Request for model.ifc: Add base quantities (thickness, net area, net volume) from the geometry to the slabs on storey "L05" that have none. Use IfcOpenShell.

First a look at what the model holds.

```python
import ifcopenshell
import ifcopenshell.util.element
import ifcopenshell.util.unit

model = ifcopenshell.open("model.ifc")
print(model.schema)
for unit_type in ("LENGTHUNIT", "AREAUNIT", "VOLUMEUNIT"):
    print(unit_type, ifcopenshell.util.unit.calculate_unit_scale(model, unit_type))
storey = next(s for s in model.by_type("IfcBuildingStorey") if s.Name == "L05")
slabs = [e for e in ifcopenshell.util.element.get_decomposition(storey) if e.is_a("IfcSlab")]
for e in sorted(slabs, key=lambda e: e.id()):
    print(e.id(), e.is_a(), e.Name, list(ifcopenshell.util.element.get_psets(e, qtos_only=True)), sep=" | ")
```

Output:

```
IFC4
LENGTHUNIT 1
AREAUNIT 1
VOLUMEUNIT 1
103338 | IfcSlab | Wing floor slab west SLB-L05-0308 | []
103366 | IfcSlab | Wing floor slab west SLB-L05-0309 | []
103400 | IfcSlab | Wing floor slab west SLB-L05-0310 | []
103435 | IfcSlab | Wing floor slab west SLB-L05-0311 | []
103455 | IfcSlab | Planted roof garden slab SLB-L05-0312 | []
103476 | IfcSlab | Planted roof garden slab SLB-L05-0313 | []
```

```python
import ifcopenshell
import ifcopenshell.api.pset
import ifcopenshell.geom
import ifcopenshell.util.element
import ifcopenshell.util.shape
import ifcopenshell.util.unit

model = ifcopenshell.open("model.ifc")
unit_scale = ifcopenshell.util.unit.calculate_unit_scale(model)
area_scale = ifcopenshell.util.unit.calculate_unit_scale(model, "AREAUNIT")
volume_scale = ifcopenshell.util.unit.calculate_unit_scale(model, "VOLUMEUNIT")
settings = ifcopenshell.geom.settings()

storey = next(s for s in model.by_type("IfcBuildingStorey") if s.Name == "L05")
slabs = [e for e in ifcopenshell.util.element.get_decomposition(storey) if e.is_a("IfcSlab")]

for e in sorted(slabs, key=lambda e: e.id()):
    if ifcopenshell.util.element.get_psets(e, qtos_only=True, should_inherit=False):
        continue
    # Geometry comes back in metres, in the element's own axes.
    shape = ifcopenshell.geom.create_shape(settings, e)
    values = {
        "Width": ifcopenshell.util.shape.get_z(shape.geometry) / unit_scale,
        "NetArea": ifcopenshell.util.shape.get_footprint_area(shape.geometry) / area_scale,
        "NetVolume": ifcopenshell.util.shape.get_volume(shape.geometry) / volume_scale,
    }
    qto = ifcopenshell.api.pset.add_qto(model, product=e, name="Qto_SlabBaseQuantities")
    ifcopenshell.api.pset.edit_qto(model, qto=qto, properties=values)
    print(e.id(), {k: round(v, 3) for k, v in values.items()})

model.write("model-out.ifc")
```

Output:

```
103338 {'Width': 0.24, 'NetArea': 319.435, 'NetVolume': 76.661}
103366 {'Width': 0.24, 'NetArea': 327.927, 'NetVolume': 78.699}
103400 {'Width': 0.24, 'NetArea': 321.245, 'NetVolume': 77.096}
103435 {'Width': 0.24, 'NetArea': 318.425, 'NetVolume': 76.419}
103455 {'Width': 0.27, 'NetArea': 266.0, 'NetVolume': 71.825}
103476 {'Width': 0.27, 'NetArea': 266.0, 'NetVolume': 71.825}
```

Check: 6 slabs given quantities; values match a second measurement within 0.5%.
